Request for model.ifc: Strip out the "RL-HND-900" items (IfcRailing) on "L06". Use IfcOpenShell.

First a look at what the model holds.

```python
import ifcopenshell
import ifcopenshell.util.element

model = ifcopenshell.open("model.ifc")
print(model.schema)
storey = next(s for s in model.by_type("IfcBuildingStorey") if s.Name == "L06")
railings = [e for e in ifcopenshell.util.element.get_decomposition(storey) if e.is_a("IfcRailing")]
seen = {}
for e in railings:
    element_type = ifcopenshell.util.element.get_type(e)
    name = element_type.Name if element_type not in (None, e) else None
    seen[name] = seen.get(name, 0) + 1
for name, count in sorted(seen.items(), key=str):
    print(count, "x", name)
```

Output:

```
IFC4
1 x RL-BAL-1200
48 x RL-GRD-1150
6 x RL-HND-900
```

```python
import ifcopenshell
import ifcopenshell.api.root
import ifcopenshell.util.element

model = ifcopenshell.open("model.ifc")

storey = next(s for s in model.by_type("IfcBuildingStorey") if s.Name == "L06")
railings = [e for e in ifcopenshell.util.element.get_decomposition(storey) if e.is_a("IfcRailing")]
targets = [e for e in railings if (t := ifcopenshell.util.element.get_type(e)) not in (None, e) and t.Name == "RL-HND-900"]

for e in targets:
    ifcopenshell.api.root.remove_product(model, product=e)
print(len(targets), "removed")

model.write("model_v2.ifc")
```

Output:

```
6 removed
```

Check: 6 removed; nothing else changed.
